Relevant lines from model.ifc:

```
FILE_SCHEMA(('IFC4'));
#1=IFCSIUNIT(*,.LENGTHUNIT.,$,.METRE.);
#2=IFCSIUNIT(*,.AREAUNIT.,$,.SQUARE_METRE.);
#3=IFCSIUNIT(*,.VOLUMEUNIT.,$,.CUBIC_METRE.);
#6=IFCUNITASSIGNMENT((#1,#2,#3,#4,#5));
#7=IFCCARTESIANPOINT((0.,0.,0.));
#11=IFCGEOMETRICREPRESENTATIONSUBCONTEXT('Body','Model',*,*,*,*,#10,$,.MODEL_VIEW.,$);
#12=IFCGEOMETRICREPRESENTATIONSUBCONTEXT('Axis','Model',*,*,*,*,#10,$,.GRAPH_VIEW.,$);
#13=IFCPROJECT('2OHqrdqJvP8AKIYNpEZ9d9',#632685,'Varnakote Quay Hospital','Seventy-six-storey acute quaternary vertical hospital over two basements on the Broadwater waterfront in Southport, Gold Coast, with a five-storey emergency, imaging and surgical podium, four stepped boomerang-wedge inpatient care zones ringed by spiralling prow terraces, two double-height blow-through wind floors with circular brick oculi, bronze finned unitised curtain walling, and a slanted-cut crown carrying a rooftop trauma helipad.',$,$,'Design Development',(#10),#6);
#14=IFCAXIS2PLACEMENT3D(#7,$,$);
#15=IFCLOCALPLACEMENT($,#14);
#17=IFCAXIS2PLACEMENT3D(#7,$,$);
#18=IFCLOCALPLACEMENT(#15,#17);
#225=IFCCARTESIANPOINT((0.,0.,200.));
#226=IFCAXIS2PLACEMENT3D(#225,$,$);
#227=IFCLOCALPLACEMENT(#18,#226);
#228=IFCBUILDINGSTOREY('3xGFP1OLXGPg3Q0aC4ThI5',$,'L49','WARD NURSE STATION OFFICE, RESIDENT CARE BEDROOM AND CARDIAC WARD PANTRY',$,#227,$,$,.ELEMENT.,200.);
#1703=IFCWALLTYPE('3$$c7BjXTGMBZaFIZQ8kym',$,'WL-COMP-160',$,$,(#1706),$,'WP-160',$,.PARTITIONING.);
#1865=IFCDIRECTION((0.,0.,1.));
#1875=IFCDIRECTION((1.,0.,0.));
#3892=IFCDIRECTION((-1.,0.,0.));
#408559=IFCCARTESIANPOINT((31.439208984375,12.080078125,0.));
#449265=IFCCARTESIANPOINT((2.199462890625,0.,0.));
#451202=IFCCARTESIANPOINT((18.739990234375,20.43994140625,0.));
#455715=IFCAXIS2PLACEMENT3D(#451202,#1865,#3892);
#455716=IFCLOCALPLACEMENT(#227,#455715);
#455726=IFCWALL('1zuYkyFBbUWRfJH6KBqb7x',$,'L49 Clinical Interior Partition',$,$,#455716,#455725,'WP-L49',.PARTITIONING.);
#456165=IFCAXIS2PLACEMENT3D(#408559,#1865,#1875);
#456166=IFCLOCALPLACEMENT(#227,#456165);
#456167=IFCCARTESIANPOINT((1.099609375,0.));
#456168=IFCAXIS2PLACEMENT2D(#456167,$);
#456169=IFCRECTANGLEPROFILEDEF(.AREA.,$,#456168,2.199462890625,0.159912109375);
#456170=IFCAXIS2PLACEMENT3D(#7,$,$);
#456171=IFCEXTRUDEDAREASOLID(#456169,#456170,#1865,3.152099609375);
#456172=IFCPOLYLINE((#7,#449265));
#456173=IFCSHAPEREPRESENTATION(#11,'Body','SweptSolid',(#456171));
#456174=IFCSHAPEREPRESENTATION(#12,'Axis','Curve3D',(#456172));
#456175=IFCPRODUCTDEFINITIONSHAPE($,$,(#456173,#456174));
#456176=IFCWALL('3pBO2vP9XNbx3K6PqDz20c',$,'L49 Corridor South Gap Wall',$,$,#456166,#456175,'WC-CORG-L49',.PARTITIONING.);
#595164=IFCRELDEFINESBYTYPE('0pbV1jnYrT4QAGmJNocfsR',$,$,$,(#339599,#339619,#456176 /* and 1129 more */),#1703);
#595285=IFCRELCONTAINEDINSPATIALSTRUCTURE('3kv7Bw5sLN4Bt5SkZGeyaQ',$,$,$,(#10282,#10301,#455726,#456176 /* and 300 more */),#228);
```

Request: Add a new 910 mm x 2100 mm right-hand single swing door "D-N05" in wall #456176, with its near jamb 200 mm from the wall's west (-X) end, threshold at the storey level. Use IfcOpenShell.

```python
import numpy as np
import ifcopenshell
import ifcopenshell.api.feature
import ifcopenshell.api.geometry
import ifcopenshell.api.root
import ifcopenshell.api.spatial
import ifcopenshell.geom
import ifcopenshell.util.element
import ifcopenshell.util.placement
import ifcopenshell.util.representation
import ifcopenshell.util.shape
import ifcopenshell.util.unit

model = ifcopenshell.open("model.ifc")
unit_scale = ifcopenshell.util.unit.calculate_unit_scale(model)
settings = ifcopenshell.geom.settings()


def volume(element):
    """Net volume in cubic metres, openings subtracted."""
    shape = ifcopenshell.geom.create_shape(settings, element)
    return ifcopenshell.util.shape.get_volume(shape.geometry)


wall = model.by_id(456176)
storey = ifcopenshell.util.element.get_container(wall, ifc_class="IfcBuildingStorey")
context = ifcopenshell.util.representation.get_context(model, "Model", "Body", "MODEL_VIEW")
before = volume(wall)

width, height, from_end, sill = 0.91, 2.1, 0.2, 0.0  # metres

# The wall runs along its own X axis, and the end named is its -X end.
wall_shape = ifcopenshell.geom.create_shape(settings, wall)
x, y, z = ifcopenshell.util.shape.get_vertices(wall_shape.geometry).T
start = x.min() + from_end
face, thickness = float(y.min()), float(y.max() - y.min())
wall_matrix = ifcopenshell.util.placement.get_local_placement(wall.ObjectPlacement)
level = ifcopenshell.util.placement.get_local_placement(storey.ObjectPlacement)[2, 3]


def in_wall(x, y):
    """Placement at x, y metres in the wall's axes, at sill height."""
    matrix = wall_matrix.copy()
    matrix[:, 3] = wall_matrix @ np.array([x / unit_scale, y / unit_scale, 0.0, 1.0])
    matrix[2, 3] = level + sill / unit_scale
    return matrix


# Opening: a box that overshoots both wall faces by 50 mm.
opening = ifcopenshell.api.root.create_entity(model, ifc_class="IfcOpeningElement", predefined_type="OPENING")
box = ifcopenshell.api.geometry.add_wall_representation(
    model, context=context, length=width, height=height, thickness=thickness + 0.1
)
ifcopenshell.api.geometry.assign_representation(model, product=opening, representation=box)
ifcopenshell.api.geometry.edit_object_placement(model, product=opening, matrix=in_wall(start, face - 0.05), is_si=False)
ifcopenshell.api.feature.add_feature(model, feature=opening, element=wall)

door = ifcopenshell.api.root.create_entity(model, ifc_class="IfcDoor", name="D-N05", predefined_type="DOOR")
door.OverallWidth, door.OverallHeight = width / unit_scale, height / unit_scale
door.OperationType = "SINGLE_SWING_RIGHT"
body = ifcopenshell.api.geometry.add_door_representation(
    model,
    context=context,
    overall_width=door.OverallWidth,
    overall_height=door.OverallHeight,
    operation_type="SINGLE_SWING_RIGHT",
    lining_properties={"LiningDepth": thickness / unit_scale, "ThresholdDepth": thickness / unit_scale},
)
ifcopenshell.api.geometry.assign_representation(model, product=door, representation=body)
ifcopenshell.api.spatial.assign_container(model, products=[door], relating_structure=storey)
ifcopenshell.api.feature.add_filling(model, opening=opening, element=door)

# The lining spans the wall, so the door starts at the wall face.
ifcopenshell.api.geometry.edit_object_placement(model, product=door, matrix=in_wall(start, face), is_si=False)

after = volume(wall)

print(f"wall volume {before:.3f} -> {after:.3f} m3")

model.write("model_rev.ifc")
```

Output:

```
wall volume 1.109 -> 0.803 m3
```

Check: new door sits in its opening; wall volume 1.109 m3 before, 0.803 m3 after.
